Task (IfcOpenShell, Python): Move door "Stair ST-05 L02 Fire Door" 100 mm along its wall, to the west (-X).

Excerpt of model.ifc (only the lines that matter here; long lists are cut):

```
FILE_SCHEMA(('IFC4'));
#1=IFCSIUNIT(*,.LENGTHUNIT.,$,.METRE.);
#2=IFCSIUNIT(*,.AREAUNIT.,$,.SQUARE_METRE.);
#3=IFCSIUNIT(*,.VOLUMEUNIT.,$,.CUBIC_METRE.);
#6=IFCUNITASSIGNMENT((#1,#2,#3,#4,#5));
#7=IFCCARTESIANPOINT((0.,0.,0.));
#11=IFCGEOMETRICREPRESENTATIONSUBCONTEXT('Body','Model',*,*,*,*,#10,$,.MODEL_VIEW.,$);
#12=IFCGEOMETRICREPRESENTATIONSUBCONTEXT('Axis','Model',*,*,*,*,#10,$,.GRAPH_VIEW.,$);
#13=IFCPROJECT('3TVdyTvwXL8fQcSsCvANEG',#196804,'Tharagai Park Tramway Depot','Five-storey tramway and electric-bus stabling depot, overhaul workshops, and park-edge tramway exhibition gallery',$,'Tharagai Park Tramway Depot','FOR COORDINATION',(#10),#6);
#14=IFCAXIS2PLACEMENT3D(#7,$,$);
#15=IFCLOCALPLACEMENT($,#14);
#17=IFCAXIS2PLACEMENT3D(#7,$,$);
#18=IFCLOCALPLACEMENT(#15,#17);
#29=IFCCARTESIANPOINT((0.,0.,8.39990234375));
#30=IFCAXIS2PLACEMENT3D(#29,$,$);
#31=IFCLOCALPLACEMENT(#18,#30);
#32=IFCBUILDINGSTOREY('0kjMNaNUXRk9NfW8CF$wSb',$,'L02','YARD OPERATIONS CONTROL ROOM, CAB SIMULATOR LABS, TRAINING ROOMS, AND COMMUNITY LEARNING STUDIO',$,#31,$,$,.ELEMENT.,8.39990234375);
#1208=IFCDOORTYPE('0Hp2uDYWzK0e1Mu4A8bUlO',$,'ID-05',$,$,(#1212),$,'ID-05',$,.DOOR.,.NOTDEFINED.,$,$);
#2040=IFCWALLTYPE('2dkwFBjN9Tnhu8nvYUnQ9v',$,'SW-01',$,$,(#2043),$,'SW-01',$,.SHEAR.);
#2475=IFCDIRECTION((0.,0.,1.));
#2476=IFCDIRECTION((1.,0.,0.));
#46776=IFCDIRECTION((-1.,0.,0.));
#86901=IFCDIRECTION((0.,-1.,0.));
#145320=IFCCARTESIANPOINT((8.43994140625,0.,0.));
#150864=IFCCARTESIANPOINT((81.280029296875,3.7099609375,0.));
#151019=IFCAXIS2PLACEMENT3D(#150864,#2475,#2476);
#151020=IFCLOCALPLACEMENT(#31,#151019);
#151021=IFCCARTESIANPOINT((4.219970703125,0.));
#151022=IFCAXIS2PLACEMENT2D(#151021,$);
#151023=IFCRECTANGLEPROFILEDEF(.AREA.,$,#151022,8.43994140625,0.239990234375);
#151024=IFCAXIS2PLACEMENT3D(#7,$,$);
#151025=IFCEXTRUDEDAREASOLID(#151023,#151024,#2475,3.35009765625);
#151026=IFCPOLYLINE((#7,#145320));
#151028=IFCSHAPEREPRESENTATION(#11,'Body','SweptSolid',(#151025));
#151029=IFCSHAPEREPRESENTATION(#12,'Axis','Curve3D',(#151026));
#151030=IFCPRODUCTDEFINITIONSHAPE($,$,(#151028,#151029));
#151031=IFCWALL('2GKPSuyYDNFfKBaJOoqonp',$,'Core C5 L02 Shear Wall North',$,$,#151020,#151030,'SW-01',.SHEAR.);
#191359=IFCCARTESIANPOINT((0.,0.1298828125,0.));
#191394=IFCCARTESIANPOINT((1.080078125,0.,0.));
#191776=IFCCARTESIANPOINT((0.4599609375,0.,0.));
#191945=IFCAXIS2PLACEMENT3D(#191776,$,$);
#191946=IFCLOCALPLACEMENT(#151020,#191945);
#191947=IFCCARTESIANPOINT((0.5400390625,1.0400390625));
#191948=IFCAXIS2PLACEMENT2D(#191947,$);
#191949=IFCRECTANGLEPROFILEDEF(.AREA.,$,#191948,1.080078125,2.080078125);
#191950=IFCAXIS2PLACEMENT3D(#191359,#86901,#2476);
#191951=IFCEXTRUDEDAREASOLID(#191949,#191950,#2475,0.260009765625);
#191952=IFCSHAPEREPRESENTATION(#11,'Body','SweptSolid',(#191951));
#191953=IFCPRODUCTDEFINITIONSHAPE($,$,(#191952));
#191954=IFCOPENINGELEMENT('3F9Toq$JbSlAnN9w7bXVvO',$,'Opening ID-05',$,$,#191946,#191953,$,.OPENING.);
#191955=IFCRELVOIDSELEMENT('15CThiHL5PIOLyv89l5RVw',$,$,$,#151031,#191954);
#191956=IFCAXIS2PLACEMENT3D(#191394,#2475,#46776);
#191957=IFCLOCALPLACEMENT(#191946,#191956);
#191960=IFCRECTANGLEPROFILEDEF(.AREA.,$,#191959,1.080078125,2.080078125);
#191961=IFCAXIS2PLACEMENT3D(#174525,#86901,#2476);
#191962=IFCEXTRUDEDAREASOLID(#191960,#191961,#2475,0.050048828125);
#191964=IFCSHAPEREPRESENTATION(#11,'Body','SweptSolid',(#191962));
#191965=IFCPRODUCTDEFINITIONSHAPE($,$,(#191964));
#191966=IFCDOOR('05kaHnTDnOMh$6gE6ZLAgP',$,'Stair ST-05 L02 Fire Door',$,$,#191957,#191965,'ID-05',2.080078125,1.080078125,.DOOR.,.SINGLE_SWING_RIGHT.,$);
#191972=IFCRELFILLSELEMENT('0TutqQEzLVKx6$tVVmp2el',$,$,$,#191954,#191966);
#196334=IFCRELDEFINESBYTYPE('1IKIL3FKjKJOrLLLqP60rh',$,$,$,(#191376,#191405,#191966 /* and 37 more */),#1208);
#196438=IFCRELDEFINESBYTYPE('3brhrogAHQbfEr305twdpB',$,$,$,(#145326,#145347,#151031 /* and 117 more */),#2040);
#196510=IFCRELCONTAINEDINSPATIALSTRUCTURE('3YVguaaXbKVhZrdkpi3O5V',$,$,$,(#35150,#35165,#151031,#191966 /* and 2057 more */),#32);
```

```python
import ifcopenshell
import ifcopenshell.api.geometry
import ifcopenshell.util.placement

model = ifcopenshell.open("model.ifc")

door = model.by_guid("05kaHnTDnOMh$6gE6ZLAgP")
opening = door.FillsVoids[0].RelatingOpeningElement
wall = opening.VoidsElements[0].RelatingBuildingElement

wall_matrix = ifcopenshell.util.placement.get_local_placement(wall.ObjectPlacement)
shift = wall_matrix[:3, 0] * -0.1
before = ifcopenshell.util.placement.get_local_placement(door.ObjectPlacement)[:3, 3].copy()

# The door is placed relative to its opening, so it follows when the opening moves.
matrix = ifcopenshell.util.placement.get_local_placement(opening.ObjectPlacement)
matrix[:3, 3] += shift
ifcopenshell.api.geometry.edit_object_placement(
    model, product=opening, matrix=matrix, is_si=False, should_transform_children=True
)

after = ifcopenshell.util.placement.get_local_placement(door.ObjectPlacement)[:3, 3]
print("door moved by", (after - before).round(3) + 0.0)

model.write("model_rev.ifc")
```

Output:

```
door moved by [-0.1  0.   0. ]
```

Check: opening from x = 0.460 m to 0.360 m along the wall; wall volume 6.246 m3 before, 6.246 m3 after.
